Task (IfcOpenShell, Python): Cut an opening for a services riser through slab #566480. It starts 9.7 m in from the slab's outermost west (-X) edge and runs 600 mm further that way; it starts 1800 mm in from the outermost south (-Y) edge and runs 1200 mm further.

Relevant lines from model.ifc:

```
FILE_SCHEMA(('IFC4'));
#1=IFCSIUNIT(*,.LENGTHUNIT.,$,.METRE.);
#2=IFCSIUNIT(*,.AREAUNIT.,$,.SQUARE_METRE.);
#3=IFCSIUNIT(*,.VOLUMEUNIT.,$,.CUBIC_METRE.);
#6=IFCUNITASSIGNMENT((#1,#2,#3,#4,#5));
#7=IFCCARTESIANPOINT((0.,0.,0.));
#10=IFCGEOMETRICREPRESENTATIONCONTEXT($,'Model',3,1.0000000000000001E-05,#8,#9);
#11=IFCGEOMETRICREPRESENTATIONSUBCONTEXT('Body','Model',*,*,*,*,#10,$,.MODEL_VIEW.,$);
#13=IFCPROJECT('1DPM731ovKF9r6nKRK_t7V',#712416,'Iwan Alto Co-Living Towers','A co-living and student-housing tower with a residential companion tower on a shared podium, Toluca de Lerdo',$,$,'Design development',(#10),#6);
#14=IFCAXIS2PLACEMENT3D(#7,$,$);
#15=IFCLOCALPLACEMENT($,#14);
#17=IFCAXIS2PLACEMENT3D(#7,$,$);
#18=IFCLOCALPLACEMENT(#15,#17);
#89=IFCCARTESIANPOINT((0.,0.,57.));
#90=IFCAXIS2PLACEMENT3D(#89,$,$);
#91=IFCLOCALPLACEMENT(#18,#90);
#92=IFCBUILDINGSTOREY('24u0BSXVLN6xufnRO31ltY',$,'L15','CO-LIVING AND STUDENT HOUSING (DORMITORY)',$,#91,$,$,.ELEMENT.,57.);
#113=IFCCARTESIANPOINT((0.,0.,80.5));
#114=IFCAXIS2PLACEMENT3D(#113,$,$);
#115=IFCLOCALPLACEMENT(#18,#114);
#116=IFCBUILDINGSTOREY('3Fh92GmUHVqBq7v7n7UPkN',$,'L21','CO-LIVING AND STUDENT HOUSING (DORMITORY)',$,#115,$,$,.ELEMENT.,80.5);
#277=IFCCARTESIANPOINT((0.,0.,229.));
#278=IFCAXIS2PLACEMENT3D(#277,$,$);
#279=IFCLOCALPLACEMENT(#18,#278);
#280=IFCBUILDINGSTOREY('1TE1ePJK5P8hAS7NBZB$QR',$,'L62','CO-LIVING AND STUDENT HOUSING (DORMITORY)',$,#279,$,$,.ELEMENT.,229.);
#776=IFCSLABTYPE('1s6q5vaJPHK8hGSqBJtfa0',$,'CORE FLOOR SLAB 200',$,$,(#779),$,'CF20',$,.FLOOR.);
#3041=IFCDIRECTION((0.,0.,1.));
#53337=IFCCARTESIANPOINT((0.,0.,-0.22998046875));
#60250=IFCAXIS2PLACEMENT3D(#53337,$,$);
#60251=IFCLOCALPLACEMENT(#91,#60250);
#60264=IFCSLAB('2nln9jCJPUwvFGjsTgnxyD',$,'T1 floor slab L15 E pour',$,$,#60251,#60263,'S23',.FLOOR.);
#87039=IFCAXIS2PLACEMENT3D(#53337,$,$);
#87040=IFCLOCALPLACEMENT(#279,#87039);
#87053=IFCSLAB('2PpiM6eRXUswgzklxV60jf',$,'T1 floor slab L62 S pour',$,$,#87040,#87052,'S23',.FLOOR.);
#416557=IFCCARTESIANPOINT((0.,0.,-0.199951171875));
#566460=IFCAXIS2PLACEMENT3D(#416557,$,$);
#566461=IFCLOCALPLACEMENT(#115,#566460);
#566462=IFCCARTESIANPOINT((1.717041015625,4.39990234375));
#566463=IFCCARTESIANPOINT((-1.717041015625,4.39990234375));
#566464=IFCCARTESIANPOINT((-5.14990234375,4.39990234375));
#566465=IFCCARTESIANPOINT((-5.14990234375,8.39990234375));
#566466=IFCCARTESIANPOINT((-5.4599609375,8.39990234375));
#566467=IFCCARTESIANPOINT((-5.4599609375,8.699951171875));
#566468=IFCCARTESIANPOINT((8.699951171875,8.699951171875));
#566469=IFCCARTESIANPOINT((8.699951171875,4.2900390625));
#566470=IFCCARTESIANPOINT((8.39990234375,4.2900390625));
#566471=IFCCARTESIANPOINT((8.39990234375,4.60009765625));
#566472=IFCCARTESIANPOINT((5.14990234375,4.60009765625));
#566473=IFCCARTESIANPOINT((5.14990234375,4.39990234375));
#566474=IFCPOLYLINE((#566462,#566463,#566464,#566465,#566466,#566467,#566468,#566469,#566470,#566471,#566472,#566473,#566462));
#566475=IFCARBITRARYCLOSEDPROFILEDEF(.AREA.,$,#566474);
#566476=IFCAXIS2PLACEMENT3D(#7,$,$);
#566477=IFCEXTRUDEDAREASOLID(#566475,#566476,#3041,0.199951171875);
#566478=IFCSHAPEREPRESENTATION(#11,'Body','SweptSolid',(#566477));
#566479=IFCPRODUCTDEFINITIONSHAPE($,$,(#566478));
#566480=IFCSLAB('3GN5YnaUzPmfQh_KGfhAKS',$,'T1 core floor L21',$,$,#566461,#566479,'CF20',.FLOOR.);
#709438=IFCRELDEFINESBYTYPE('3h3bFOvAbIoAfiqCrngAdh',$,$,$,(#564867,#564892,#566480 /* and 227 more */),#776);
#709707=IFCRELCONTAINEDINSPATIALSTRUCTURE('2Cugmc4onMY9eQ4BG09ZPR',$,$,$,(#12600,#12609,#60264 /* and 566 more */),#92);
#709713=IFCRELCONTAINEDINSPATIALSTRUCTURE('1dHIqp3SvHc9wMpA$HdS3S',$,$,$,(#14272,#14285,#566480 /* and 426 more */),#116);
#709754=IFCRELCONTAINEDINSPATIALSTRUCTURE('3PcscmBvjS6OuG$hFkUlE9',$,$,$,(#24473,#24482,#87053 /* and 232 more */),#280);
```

```python
import numpy as np
import ifcopenshell
import ifcopenshell.api.feature
import ifcopenshell.api.geometry
import ifcopenshell.api.root
import ifcopenshell.geom
import ifcopenshell.util.placement
import ifcopenshell.util.representation
import ifcopenshell.util.shape
import ifcopenshell.util.unit

model = ifcopenshell.open("model.ifc")
unit_scale = ifcopenshell.util.unit.calculate_unit_scale(model)
settings = ifcopenshell.geom.settings()


def volume(element):
    """Net volume in cubic metres, openings subtracted."""
    shape = ifcopenshell.geom.create_shape(settings, element)
    return ifcopenshell.util.shape.get_volume(shape.geometry)


slab = model.by_guid("3GN5YnaUzPmfQh_KGfhAKS")
before = volume(slab)

# Extent in the slab's own axes, in metres. The edges named are its -X and -Y sides.
slab_shape = ifcopenshell.geom.create_shape(settings, slab)
vertices = ifcopenshell.util.shape.get_vertices(slab_shape.geometry)
x_min, y_min, bottom = vertices.min(axis=0)
top = vertices[:, 2].max()

opening = ifcopenshell.api.root.create_entity(model, ifc_class="IfcOpeningElement", name="Services riser opening", predefined_type="OPENING")
context = ifcopenshell.util.representation.get_context(model, "Model", "Body", "MODEL_VIEW")
width, depth = 0.6, 1.2
outline = [(0.0, 0.0), (width, 0.0), (width, depth), (0.0, depth), (0.0, 0.0)]
# Overshoot both faces by 50 mm so the cut is clean.
shape = ifcopenshell.api.geometry.add_slab_representation(
    model, context=context, depth=top - bottom + 0.1, polyline=outline
)
ifcopenshell.api.geometry.assign_representation(model, product=opening, representation=shape)

matrix = ifcopenshell.util.placement.get_local_placement(slab.ObjectPlacement)
matrix[:, 3] = matrix @ np.append(np.array([x_min + 9.7, y_min + 1.8, bottom - 0.05]) / unit_scale, 1.0)
ifcopenshell.api.geometry.edit_object_placement(model, product=opening, matrix=matrix, is_si=False)
ifcopenshell.api.feature.add_feature(model, feature=opening, element=slab)

after = volume(slab)

print(f"slab volume {before:.3f} -> {after:.3f} m3")

model.write("model_rev.ifc")
```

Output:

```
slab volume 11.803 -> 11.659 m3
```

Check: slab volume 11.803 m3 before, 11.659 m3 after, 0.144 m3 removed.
